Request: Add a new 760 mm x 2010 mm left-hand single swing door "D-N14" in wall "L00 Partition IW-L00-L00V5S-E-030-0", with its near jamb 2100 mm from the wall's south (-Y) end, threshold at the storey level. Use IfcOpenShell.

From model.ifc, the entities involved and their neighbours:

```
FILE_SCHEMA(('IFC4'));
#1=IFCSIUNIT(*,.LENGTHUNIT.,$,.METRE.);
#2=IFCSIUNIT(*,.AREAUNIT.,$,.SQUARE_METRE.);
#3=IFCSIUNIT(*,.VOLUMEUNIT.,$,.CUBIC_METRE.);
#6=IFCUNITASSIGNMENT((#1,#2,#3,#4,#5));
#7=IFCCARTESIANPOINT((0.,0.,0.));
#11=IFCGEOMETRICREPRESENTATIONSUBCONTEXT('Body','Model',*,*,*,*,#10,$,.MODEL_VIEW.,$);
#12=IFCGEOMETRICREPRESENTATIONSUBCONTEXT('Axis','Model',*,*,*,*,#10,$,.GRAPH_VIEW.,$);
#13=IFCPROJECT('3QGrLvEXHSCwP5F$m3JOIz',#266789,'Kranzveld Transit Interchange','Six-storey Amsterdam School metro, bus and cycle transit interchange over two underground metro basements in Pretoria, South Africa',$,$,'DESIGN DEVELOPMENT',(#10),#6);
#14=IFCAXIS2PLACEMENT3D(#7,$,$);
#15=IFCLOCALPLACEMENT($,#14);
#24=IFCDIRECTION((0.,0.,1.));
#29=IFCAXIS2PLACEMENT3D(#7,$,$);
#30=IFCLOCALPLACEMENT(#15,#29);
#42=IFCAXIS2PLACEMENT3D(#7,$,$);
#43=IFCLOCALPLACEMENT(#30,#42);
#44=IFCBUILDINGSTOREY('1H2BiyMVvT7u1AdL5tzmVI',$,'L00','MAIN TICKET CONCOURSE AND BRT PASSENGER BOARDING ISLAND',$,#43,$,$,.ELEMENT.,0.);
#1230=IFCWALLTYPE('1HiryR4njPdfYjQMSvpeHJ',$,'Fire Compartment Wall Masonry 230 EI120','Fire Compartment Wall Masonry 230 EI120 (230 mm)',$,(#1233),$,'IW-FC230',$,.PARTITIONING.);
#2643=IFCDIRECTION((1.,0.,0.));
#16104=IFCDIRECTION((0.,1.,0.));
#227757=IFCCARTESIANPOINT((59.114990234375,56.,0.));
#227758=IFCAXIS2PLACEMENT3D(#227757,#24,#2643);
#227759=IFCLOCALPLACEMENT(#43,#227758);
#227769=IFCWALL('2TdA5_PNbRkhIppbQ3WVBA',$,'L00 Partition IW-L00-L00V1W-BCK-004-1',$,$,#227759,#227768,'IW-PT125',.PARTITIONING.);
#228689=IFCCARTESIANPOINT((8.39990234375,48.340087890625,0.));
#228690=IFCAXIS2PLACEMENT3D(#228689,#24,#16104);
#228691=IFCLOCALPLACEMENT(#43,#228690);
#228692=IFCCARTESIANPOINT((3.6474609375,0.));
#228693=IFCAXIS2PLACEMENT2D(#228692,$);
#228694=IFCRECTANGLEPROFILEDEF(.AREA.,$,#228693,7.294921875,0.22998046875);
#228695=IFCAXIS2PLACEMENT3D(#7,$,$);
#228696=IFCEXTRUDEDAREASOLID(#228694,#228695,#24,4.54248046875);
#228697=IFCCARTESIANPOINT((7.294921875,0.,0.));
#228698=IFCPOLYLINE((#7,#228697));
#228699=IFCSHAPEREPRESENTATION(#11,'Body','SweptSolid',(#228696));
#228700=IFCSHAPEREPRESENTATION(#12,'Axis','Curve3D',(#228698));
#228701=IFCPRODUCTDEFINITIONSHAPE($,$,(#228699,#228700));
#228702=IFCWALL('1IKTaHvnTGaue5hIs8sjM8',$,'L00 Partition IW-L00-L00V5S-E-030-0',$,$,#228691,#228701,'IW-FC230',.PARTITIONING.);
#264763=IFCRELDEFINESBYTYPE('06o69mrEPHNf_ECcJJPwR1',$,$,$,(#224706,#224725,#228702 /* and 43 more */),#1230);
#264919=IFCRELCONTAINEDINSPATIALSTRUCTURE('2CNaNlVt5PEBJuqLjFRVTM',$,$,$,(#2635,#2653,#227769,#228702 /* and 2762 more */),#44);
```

```python
import numpy as np
import ifcopenshell
import ifcopenshell.api.feature
import ifcopenshell.api.geometry
import ifcopenshell.api.root
import ifcopenshell.api.spatial
import ifcopenshell.geom
import ifcopenshell.util.element
import ifcopenshell.util.placement
import ifcopenshell.util.representation
import ifcopenshell.util.shape
import ifcopenshell.util.unit

model = ifcopenshell.open("model.ifc")
unit_scale = ifcopenshell.util.unit.calculate_unit_scale(model)
settings = ifcopenshell.geom.settings()


def volume(element):
    """Net volume in cubic metres, openings subtracted."""
    shape = ifcopenshell.geom.create_shape(settings, element)
    return ifcopenshell.util.shape.get_volume(shape.geometry)


wall = model.by_guid("1IKTaHvnTGaue5hIs8sjM8")
storey = ifcopenshell.util.element.get_container(wall, ifc_class="IfcBuildingStorey")
context = ifcopenshell.util.representation.get_context(model, "Model", "Body", "MODEL_VIEW")
before = volume(wall)

width, height, from_end, sill = 0.76, 2.01, 2.1, 0.0  # metres

# The wall runs along its own X axis, and the end named is its -X end.
wall_shape = ifcopenshell.geom.create_shape(settings, wall)
x, y, z = ifcopenshell.util.shape.get_vertices(wall_shape.geometry).T
start = x.min() + from_end
face, thickness = float(y.min()), float(y.max() - y.min())
wall_matrix = ifcopenshell.util.placement.get_local_placement(wall.ObjectPlacement)
level = ifcopenshell.util.placement.get_local_placement(storey.ObjectPlacement)[2, 3]


def in_wall(x, y):
    """Placement at x, y metres in the wall's axes, at sill height."""
    matrix = wall_matrix.copy()
    matrix[:, 3] = wall_matrix @ np.array([x / unit_scale, y / unit_scale, 0.0, 1.0])
    matrix[2, 3] = level + sill / unit_scale
    return matrix


# Opening: a box that overshoots both wall faces by 50 mm.
opening = ifcopenshell.api.root.create_entity(model, ifc_class="IfcOpeningElement", predefined_type="OPENING")
box = ifcopenshell.api.geometry.add_wall_representation(
    model, context=context, length=width, height=height, thickness=thickness + 0.1
)
ifcopenshell.api.geometry.assign_representation(model, product=opening, representation=box)
ifcopenshell.api.geometry.edit_object_placement(model, product=opening, matrix=in_wall(start, face - 0.05), is_si=False)
ifcopenshell.api.feature.add_feature(model, feature=opening, element=wall)

door = ifcopenshell.api.root.create_entity(model, ifc_class="IfcDoor", name="D-N14", predefined_type="DOOR")
door.OverallWidth, door.OverallHeight = width / unit_scale, height / unit_scale
door.OperationType = "SINGLE_SWING_LEFT"
body = ifcopenshell.api.geometry.add_door_representation(
    model,
    context=context,
    overall_width=door.OverallWidth,
    overall_height=door.OverallHeight,
    operation_type="SINGLE_SWING_LEFT",
    lining_properties={"LiningDepth": thickness / unit_scale, "ThresholdDepth": thickness / unit_scale},
)
ifcopenshell.api.geometry.assign_representation(model, product=door, representation=body)
ifcopenshell.api.spatial.assign_container(model, products=[door], relating_structure=storey)
ifcopenshell.api.feature.add_filling(model, opening=opening, element=door)

# The lining spans the wall, so the door starts at the wall face.
ifcopenshell.api.geometry.edit_object_placement(model, product=door, matrix=in_wall(start, face), is_si=False)

after = volume(wall)

print(f"wall volume {before:.3f} -> {after:.3f} m3")

model.write("model-out.ifc")
```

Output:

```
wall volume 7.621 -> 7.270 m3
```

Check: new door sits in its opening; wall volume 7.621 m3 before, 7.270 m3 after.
